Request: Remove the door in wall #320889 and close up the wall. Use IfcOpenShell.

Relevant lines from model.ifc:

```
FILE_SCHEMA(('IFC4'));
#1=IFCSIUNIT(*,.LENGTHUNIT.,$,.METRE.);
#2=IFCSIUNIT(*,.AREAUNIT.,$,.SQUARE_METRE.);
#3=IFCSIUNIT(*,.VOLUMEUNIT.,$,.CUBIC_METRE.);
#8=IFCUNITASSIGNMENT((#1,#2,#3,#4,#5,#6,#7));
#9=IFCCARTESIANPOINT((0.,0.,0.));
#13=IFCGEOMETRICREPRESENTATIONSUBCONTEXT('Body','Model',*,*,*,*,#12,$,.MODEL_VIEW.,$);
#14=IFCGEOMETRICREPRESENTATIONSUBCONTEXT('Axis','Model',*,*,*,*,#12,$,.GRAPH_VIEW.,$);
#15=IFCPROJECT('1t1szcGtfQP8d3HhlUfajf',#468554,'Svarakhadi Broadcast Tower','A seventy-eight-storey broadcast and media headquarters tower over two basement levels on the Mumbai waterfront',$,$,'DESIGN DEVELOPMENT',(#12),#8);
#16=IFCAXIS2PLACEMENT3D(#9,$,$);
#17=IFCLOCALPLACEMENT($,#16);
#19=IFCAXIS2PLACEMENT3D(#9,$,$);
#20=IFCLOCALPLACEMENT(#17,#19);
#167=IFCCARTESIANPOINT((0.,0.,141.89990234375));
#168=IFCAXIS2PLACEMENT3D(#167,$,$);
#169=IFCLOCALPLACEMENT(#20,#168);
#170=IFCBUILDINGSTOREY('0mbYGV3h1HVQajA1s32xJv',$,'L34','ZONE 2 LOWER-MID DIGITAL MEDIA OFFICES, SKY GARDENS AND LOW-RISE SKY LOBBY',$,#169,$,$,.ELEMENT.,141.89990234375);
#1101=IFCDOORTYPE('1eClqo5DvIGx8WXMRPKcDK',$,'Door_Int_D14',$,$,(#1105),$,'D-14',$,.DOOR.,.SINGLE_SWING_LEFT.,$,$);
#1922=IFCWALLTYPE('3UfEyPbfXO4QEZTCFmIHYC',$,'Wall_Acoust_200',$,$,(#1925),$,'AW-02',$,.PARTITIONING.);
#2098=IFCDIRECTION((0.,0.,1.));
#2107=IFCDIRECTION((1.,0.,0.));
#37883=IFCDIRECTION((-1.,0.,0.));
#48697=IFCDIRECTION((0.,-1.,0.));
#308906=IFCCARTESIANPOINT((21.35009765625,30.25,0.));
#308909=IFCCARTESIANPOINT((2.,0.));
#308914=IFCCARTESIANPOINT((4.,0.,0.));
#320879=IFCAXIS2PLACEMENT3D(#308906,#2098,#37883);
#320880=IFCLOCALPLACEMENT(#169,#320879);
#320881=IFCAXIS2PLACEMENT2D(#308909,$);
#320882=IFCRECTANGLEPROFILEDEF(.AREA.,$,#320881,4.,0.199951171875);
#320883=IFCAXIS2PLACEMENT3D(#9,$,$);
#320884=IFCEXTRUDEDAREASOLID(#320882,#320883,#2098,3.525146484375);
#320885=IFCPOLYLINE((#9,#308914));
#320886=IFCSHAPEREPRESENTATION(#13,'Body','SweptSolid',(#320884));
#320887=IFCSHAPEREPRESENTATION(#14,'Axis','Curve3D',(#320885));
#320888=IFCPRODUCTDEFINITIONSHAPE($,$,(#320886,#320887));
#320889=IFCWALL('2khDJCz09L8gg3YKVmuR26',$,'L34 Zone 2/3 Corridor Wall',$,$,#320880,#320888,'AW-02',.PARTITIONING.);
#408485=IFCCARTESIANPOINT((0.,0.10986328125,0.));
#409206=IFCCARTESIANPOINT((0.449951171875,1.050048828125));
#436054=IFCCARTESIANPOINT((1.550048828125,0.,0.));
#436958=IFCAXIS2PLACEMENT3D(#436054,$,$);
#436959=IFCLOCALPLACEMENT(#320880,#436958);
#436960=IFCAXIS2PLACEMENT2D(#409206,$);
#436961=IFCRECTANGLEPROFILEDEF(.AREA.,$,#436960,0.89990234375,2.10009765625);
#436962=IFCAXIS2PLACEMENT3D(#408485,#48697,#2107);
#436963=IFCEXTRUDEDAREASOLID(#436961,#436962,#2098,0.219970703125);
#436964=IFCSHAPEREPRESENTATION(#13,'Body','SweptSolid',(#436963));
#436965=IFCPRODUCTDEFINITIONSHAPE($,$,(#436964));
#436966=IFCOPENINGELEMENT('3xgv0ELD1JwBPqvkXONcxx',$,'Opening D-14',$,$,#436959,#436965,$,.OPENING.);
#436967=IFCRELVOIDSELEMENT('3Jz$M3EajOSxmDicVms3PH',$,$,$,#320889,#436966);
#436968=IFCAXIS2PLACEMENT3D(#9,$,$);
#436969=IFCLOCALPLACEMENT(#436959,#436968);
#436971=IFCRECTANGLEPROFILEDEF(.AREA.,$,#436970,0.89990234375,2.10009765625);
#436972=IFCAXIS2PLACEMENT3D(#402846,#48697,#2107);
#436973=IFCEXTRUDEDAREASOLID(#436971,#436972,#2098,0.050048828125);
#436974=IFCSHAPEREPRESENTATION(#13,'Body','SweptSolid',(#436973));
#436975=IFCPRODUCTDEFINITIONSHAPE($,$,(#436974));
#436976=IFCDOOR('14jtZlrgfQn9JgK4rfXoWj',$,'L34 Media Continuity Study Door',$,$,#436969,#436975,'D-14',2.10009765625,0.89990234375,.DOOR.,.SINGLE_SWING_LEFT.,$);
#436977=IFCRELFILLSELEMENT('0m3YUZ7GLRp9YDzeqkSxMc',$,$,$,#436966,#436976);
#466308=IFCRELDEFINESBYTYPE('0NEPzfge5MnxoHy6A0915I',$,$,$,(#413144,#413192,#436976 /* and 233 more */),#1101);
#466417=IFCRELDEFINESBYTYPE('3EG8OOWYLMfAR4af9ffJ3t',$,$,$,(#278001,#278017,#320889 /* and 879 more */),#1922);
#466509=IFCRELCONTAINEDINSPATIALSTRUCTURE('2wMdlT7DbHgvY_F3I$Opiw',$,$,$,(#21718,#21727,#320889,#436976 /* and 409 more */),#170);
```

```python
import ifcopenshell
import ifcopenshell.api.feature
import ifcopenshell.api.root
import ifcopenshell.geom
import ifcopenshell.util.shape

model = ifcopenshell.open("model.ifc")
settings = ifcopenshell.geom.settings()


def volume(element):
    """Net volume in cubic metres, openings subtracted."""
    shape = ifcopenshell.geom.create_shape(settings, element)
    return ifcopenshell.util.shape.get_volume(shape.geometry)


door = model.by_guid("14jtZlrgfQn9JgK4rfXoWj")
opening = door.FillsVoids[0].RelatingOpeningElement
wall = opening.VoidsElements[0].RelatingBuildingElement
before = volume(wall)

ifcopenshell.api.root.remove_product(model, product=door)
ifcopenshell.api.feature.remove_feature(model, feature=opening)

after = volume(wall)

print(f"wall volume {before:.3f} -> {after:.3f} m3")

model.write("model_v2.ifc")
```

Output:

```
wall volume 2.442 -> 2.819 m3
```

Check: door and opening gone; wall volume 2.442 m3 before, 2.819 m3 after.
